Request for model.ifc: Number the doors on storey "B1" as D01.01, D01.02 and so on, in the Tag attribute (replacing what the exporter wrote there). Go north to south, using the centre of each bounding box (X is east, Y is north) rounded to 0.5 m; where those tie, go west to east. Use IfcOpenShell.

First a look at what the model holds.

```python
import ifcopenshell
import ifcopenshell.util.element
import ifcopenshell.util.placement

model = ifcopenshell.open("model.ifc")
print(model.schema)
storey = next(s for s in model.by_type("IfcBuildingStorey") if s.Name == "B1")
doors = [e for e in ifcopenshell.util.element.get_decomposition(storey) if e.is_a("IfcDoor")]
for e in sorted(doors, key=lambda e: e.id()):
    origin = ifcopenshell.util.placement.get_local_placement(e.ObjectPlacement)[:3, 3]
    print(e.id(), e.Tag, e.Name, origin.round(2) + 0.0, sep=" | ")
```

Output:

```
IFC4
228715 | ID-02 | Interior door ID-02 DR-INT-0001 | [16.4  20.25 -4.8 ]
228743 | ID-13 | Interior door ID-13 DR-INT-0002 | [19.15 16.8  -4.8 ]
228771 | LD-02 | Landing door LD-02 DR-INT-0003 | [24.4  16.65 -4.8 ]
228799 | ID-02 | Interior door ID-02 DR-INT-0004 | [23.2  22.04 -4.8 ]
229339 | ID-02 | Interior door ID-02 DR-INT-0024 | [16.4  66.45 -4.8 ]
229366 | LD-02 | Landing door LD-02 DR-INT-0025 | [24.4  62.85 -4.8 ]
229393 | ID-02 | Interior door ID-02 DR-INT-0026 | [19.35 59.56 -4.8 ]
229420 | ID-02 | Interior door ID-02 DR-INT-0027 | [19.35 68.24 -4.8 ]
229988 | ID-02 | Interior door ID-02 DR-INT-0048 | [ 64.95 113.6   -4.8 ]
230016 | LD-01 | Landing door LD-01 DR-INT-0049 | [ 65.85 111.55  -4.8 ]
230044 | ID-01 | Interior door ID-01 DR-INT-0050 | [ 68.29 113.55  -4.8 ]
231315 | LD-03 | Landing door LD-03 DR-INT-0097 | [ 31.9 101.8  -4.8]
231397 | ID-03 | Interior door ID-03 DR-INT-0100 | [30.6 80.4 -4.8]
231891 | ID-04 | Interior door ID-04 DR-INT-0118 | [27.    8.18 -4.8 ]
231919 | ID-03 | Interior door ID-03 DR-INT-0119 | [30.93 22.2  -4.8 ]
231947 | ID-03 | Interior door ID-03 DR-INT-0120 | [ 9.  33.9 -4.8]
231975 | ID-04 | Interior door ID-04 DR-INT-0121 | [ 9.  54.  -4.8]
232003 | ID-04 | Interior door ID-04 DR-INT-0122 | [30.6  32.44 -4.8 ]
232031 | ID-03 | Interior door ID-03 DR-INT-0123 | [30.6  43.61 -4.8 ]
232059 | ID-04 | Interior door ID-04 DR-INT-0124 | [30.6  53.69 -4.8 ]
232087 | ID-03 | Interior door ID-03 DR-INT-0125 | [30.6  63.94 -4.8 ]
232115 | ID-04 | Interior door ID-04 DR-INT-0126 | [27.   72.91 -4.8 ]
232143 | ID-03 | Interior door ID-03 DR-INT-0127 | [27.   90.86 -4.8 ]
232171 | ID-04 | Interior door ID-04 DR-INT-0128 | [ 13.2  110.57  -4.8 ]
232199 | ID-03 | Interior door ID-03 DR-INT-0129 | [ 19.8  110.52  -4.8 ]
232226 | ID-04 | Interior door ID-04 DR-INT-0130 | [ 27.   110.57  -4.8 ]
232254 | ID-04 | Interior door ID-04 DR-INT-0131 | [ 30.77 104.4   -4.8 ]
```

```python
import ifcopenshell
import ifcopenshell.geom
import ifcopenshell.util.element
import ifcopenshell.util.shape

model = ifcopenshell.open("model.ifc")
settings = ifcopenshell.geom.settings()
settings.set("use-world-coords", True)


def centre(element):
    shape = ifcopenshell.geom.create_shape(settings, element)
    return ifcopenshell.util.shape.get_bbox_centroid(shape.geometry)


storey = next(s for s in model.by_type("IfcBuildingStorey") if s.Name == "B1")
doors = [e for e in ifcopenshell.util.element.get_decomposition(storey) if e.is_a("IfcDoor")]

# Insertion points can sit at a corner or the storey origin, so sort by the geometry (in metres).
centres = {e: centre(e) for e in doors}
doors.sort(key=lambda e: (-round(centres[e][1] / 0.5), centres[e][0]))

for i, e in enumerate(doors, start=1):
    number = f"D01.{i:02d}"
    e.Tag = number
    print(e.id(), number)

model.write("model_updated.ifc")
```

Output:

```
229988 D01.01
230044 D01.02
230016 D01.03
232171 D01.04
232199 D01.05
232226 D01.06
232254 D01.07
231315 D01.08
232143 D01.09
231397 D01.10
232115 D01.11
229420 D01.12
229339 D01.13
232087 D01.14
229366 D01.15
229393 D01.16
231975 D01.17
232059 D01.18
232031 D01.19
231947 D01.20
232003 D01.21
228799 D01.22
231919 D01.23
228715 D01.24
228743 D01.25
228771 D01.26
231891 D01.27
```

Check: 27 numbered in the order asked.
